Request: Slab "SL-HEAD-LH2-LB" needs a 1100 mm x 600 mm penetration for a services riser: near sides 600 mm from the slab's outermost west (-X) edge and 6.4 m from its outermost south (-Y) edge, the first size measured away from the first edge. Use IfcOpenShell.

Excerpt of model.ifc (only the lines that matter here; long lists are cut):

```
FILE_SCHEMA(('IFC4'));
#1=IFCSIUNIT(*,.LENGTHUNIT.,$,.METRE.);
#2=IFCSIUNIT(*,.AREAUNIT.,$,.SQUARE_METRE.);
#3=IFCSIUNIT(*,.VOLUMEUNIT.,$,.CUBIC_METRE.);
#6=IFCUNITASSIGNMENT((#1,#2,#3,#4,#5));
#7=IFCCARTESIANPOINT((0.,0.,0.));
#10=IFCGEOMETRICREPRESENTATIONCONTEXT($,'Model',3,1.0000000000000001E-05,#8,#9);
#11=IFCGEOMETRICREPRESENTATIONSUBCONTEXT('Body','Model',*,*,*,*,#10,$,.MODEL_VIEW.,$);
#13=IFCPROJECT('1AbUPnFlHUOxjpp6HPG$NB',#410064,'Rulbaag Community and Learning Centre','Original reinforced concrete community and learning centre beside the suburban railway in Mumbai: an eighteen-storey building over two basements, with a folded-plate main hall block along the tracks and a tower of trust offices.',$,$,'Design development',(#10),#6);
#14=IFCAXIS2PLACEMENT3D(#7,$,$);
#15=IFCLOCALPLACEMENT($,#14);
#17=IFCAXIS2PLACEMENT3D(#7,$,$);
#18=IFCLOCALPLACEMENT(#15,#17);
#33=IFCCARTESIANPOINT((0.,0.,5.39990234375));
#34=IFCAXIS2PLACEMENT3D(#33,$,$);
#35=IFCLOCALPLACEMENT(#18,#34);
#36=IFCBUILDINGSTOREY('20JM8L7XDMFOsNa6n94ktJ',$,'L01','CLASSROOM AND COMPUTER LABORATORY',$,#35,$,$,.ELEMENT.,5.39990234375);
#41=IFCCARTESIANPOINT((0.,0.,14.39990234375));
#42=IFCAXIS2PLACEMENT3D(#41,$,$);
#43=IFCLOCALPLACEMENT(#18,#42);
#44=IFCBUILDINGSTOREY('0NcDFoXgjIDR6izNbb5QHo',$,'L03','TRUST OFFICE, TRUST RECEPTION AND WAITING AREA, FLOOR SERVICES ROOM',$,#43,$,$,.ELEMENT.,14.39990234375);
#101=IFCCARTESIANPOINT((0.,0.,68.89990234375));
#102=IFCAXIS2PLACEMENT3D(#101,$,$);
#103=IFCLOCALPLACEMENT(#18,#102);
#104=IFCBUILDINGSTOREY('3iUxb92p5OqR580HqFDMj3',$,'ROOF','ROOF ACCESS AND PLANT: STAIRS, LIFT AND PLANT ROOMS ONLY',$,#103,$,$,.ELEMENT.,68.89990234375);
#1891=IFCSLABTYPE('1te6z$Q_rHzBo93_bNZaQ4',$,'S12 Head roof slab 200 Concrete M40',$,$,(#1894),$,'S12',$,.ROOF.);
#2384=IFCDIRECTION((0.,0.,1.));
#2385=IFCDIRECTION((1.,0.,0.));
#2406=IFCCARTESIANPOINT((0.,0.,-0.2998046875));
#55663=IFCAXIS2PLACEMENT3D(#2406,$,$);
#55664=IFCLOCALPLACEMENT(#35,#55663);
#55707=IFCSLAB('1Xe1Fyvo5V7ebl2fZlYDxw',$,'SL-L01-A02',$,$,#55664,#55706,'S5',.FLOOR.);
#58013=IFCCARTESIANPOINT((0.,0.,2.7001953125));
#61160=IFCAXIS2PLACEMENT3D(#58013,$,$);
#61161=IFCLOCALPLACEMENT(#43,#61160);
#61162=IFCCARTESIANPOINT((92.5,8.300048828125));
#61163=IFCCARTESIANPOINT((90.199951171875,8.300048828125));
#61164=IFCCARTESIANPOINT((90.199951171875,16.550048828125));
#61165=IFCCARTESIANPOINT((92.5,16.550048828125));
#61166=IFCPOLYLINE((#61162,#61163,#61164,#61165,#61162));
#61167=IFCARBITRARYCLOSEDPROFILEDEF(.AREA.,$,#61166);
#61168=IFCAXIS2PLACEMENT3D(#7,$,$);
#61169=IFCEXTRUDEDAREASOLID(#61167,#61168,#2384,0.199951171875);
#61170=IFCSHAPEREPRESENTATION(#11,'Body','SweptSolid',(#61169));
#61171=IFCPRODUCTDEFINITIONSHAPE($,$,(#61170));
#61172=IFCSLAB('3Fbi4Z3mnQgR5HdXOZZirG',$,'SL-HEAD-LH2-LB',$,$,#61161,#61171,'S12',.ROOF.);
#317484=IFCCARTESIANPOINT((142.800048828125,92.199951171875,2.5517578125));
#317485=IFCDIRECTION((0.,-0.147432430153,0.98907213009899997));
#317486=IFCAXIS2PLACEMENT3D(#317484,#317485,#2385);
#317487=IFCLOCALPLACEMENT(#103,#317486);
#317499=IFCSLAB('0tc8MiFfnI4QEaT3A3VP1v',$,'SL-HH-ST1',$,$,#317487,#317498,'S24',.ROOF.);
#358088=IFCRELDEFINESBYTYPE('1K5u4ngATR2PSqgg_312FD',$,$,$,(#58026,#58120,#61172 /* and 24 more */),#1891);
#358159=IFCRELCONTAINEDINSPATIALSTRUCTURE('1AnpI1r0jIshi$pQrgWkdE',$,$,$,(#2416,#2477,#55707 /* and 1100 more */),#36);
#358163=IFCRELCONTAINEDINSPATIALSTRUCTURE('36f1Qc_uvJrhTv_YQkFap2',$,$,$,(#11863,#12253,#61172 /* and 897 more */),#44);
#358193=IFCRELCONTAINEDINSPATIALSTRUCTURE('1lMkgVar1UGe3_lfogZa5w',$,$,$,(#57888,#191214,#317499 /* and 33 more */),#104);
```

```python
import numpy as np
import ifcopenshell
import ifcopenshell.api.feature
import ifcopenshell.api.geometry
import ifcopenshell.api.root
import ifcopenshell.geom
import ifcopenshell.util.placement
import ifcopenshell.util.representation
import ifcopenshell.util.shape
import ifcopenshell.util.unit

model = ifcopenshell.open("model.ifc")
unit_scale = ifcopenshell.util.unit.calculate_unit_scale(model)
settings = ifcopenshell.geom.settings()


def volume(element):
    """Net volume in cubic metres, openings subtracted."""
    shape = ifcopenshell.geom.create_shape(settings, element)
    return ifcopenshell.util.shape.get_volume(shape.geometry)


slab = model.by_guid("3Fbi4Z3mnQgR5HdXOZZirG")
before = volume(slab)

# Extent in the slab's own axes, in metres. The edges named are its -X and -Y sides.
slab_shape = ifcopenshell.geom.create_shape(settings, slab)
vertices = ifcopenshell.util.shape.get_vertices(slab_shape.geometry)
x_min, y_min, bottom = vertices.min(axis=0)
top = vertices[:, 2].max()

opening = ifcopenshell.api.root.create_entity(model, ifc_class="IfcOpeningElement", name="Services riser opening", predefined_type="OPENING")
context = ifcopenshell.util.representation.get_context(model, "Model", "Body", "MODEL_VIEW")
width, depth = 1.1, 0.6
outline = [(0.0, 0.0), (width, 0.0), (width, depth), (0.0, depth), (0.0, 0.0)]
# Overshoot both faces by 50 mm so the cut is clean.
shape = ifcopenshell.api.geometry.add_slab_representation(
    model, context=context, depth=top - bottom + 0.1, polyline=outline
)
ifcopenshell.api.geometry.assign_representation(model, product=opening, representation=shape)

matrix = ifcopenshell.util.placement.get_local_placement(slab.ObjectPlacement)
matrix[:, 3] = matrix @ np.append(np.array([x_min + 0.6, y_min + 6.4, bottom - 0.05]) / unit_scale, 1.0)
ifcopenshell.api.geometry.edit_object_placement(model, product=opening, matrix=matrix, is_si=False)
ifcopenshell.api.feature.add_feature(model, feature=opening, element=slab)

after = volume(slab)

print(f"slab volume {before:.3f} -> {after:.3f} m3")

model.write("model_updated.ifc")
```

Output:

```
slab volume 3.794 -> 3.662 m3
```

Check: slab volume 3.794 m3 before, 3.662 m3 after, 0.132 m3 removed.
